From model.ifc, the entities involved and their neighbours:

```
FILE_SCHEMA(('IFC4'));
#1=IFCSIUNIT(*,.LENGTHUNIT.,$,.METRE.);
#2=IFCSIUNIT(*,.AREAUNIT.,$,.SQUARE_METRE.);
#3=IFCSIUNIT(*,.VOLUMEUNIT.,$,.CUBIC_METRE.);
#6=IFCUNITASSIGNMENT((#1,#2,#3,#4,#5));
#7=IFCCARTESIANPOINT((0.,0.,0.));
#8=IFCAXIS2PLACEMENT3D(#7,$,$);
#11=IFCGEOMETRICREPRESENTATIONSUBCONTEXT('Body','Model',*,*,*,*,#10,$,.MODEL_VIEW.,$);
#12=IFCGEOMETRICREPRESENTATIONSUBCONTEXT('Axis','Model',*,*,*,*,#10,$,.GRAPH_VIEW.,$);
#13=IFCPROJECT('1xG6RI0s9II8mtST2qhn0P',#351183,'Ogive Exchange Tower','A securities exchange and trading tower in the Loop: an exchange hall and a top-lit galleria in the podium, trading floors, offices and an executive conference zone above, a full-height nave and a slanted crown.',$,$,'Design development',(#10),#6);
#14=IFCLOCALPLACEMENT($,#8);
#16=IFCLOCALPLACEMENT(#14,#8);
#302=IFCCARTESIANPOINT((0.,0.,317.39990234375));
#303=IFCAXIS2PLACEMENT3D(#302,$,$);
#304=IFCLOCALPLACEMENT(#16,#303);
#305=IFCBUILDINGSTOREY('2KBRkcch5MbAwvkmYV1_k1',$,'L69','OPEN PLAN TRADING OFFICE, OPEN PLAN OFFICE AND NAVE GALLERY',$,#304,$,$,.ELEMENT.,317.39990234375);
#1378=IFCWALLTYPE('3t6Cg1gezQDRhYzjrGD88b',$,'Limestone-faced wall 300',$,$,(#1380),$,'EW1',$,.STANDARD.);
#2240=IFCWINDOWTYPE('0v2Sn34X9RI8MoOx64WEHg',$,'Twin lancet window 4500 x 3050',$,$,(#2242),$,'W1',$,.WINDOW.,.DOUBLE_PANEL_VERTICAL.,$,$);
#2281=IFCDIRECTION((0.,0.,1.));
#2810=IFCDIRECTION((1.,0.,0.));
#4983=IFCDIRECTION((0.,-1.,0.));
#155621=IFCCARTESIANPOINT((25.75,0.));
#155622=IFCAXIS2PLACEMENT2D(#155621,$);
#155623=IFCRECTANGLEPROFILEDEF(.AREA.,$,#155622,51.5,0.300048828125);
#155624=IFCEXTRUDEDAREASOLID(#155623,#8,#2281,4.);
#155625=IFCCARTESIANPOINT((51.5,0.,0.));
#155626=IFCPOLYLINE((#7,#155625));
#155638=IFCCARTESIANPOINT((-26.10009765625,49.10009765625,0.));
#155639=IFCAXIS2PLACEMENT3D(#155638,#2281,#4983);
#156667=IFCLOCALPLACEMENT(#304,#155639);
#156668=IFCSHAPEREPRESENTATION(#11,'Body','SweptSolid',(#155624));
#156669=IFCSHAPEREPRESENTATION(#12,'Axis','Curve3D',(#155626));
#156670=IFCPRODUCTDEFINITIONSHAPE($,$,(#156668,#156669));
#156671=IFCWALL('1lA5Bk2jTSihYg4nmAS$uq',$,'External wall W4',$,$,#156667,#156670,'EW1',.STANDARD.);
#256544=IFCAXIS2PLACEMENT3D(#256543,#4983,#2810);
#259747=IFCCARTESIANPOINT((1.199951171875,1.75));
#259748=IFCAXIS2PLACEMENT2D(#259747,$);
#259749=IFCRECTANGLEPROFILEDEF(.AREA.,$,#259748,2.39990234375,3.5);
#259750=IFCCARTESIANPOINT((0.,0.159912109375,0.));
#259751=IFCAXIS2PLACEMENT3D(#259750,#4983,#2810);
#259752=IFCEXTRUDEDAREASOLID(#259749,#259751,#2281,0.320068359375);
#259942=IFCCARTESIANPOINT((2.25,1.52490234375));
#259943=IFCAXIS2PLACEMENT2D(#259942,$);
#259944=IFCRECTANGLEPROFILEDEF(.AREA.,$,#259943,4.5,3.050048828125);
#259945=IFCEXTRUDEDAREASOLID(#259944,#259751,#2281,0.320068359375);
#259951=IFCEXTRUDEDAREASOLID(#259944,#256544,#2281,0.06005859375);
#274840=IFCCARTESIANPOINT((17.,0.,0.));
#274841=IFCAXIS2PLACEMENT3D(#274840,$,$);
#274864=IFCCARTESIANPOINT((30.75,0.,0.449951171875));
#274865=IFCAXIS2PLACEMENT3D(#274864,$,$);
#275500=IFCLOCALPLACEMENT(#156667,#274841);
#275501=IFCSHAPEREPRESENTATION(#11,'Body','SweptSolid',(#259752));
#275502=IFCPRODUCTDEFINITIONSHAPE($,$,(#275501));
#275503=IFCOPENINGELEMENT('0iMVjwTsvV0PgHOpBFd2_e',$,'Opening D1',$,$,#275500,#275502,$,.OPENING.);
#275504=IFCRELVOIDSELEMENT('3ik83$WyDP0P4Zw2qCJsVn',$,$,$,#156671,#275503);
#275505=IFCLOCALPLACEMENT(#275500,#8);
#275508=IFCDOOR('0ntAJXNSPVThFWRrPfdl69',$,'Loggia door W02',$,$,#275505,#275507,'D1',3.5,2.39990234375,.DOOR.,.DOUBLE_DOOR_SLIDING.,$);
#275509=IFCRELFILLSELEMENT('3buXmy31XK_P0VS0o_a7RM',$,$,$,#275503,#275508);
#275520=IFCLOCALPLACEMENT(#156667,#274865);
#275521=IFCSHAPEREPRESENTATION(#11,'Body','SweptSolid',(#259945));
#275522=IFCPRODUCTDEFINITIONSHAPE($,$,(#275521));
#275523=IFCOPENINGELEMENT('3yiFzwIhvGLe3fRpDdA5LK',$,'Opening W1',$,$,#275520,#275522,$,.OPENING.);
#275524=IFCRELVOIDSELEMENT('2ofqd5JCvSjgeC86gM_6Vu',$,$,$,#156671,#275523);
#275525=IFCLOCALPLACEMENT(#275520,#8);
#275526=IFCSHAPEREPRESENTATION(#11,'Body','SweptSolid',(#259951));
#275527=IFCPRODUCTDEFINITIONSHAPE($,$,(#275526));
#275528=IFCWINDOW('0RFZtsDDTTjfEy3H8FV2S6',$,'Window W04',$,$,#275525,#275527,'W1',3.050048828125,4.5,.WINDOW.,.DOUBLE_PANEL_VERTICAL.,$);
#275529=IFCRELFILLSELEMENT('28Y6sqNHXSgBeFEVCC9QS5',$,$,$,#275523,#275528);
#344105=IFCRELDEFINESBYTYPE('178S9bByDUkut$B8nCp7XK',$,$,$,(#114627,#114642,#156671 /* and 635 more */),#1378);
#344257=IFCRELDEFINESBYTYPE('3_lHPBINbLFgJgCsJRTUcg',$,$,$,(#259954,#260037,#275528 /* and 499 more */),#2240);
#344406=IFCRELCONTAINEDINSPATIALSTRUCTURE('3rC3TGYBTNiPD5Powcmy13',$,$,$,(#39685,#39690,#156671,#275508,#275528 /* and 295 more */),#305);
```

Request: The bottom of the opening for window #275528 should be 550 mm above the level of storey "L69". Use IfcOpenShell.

```python
import numpy as np
import ifcopenshell
import ifcopenshell.api.geometry
import ifcopenshell.geom
import ifcopenshell.util.element
import ifcopenshell.util.placement
import ifcopenshell.util.shape
import ifcopenshell.util.unit

model = ifcopenshell.open("model.ifc")
unit_scale = ifcopenshell.util.unit.calculate_unit_scale(model)

window = model.by_id(275528)
opening = window.FillsVoids[0].RelatingOpeningElement
storey = ifcopenshell.util.element.get_container(window, ifc_class="IfcBuildingStorey")
level = ifcopenshell.util.placement.get_local_placement(storey.ObjectPlacement)[2, 3]

# The opening's origin need not be at the sill, so measure its lowest point.
shape = ifcopenshell.geom.create_shape(ifcopenshell.geom.settings(), opening)
bottom = ifcopenshell.util.shape.get_shape_bottom_elevation(shape, shape.geometry) / unit_scale
dz = level + 0.55 - bottom

shift = np.array([0.0, 0.0, dz])
# The window is placed relative to its opening, so it follows when the opening moves.
matrix = ifcopenshell.util.placement.get_local_placement(opening.ObjectPlacement)
matrix[:3, 3] += shift
ifcopenshell.api.geometry.edit_object_placement(
    model, product=opening, matrix=matrix, is_si=False, should_transform_children=True
)

print(f"moved by {dz * unit_scale:+.3f} m")

model.write("model-out.ifc")
```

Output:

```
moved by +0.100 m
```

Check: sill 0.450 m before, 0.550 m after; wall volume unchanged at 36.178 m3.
